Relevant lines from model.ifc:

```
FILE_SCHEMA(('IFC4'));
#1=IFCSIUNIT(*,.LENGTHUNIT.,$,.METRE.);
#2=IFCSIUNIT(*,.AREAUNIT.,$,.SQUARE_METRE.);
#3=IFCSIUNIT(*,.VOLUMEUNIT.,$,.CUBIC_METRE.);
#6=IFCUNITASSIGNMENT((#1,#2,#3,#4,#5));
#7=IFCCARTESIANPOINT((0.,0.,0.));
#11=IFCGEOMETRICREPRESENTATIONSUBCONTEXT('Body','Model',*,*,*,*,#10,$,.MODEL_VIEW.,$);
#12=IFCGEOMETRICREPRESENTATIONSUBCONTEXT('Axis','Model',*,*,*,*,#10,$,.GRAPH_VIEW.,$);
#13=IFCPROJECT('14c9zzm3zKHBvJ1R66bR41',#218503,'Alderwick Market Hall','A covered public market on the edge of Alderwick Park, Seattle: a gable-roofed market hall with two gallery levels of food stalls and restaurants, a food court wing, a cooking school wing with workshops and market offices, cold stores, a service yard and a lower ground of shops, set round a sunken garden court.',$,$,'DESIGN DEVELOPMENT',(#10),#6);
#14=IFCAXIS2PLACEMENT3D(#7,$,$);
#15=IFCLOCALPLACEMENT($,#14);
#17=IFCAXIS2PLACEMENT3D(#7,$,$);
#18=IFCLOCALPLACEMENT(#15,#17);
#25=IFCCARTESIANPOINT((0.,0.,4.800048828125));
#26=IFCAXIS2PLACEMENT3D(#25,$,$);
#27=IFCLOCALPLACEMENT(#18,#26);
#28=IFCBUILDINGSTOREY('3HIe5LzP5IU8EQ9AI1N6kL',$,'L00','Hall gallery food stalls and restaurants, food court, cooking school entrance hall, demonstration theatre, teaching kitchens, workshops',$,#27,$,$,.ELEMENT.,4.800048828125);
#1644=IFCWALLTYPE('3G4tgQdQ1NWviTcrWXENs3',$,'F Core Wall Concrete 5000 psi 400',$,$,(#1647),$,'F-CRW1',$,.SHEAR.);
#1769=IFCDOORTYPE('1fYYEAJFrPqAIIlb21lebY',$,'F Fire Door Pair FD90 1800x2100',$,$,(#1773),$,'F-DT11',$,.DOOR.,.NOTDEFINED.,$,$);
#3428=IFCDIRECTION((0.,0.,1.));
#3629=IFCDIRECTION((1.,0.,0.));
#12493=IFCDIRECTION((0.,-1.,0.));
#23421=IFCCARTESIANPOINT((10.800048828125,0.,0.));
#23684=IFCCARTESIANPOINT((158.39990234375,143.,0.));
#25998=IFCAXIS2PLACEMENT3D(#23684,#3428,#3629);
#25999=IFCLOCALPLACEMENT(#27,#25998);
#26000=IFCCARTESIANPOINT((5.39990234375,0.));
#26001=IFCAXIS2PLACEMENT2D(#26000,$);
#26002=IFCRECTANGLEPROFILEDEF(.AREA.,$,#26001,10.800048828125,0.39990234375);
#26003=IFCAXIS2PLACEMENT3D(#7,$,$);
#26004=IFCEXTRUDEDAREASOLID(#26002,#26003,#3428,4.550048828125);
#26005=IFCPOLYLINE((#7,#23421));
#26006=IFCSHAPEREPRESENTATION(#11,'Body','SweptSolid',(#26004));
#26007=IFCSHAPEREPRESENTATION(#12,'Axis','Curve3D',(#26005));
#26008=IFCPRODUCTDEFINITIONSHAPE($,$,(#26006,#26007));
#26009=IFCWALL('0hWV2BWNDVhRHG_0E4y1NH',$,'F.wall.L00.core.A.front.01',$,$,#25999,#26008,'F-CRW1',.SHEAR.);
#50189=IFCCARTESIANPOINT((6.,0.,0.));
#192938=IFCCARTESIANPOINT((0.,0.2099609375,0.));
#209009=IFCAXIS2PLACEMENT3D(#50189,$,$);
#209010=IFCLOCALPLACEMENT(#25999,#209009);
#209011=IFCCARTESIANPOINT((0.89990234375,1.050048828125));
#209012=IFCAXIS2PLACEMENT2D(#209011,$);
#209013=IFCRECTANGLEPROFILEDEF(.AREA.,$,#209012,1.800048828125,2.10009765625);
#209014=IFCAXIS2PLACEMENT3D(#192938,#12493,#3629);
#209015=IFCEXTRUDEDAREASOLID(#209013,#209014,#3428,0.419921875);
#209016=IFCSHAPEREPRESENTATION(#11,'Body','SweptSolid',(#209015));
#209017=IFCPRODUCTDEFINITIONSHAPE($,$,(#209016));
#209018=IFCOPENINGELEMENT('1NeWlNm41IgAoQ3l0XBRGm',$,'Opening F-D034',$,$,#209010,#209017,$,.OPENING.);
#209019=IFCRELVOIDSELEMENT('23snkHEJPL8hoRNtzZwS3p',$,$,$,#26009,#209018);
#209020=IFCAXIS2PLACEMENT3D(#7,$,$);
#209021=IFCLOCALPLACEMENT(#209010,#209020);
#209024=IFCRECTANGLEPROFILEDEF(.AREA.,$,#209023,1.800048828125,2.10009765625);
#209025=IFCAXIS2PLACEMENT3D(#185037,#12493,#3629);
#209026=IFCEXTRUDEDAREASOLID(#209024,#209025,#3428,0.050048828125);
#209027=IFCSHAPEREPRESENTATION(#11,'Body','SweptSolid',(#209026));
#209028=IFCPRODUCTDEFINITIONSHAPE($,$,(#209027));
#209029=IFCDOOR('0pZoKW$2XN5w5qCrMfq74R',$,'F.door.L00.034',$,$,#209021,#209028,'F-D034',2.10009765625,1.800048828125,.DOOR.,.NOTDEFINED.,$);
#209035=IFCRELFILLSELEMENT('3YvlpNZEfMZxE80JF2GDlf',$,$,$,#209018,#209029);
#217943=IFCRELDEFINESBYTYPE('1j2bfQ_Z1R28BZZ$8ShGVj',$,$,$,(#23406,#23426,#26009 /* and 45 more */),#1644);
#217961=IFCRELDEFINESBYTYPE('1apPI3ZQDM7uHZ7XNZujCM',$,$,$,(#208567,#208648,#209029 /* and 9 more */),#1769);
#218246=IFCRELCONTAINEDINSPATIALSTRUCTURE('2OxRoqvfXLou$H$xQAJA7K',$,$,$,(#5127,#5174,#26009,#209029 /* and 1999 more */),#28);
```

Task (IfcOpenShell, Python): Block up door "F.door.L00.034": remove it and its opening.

```python
import ifcopenshell
import ifcopenshell.api.feature
import ifcopenshell.api.root
import ifcopenshell.geom
import ifcopenshell.util.shape

model = ifcopenshell.open("model.ifc")
settings = ifcopenshell.geom.settings()


def volume(element):
    """Net volume in cubic metres, openings subtracted."""
    shape = ifcopenshell.geom.create_shape(settings, element)
    return ifcopenshell.util.shape.get_volume(shape.geometry)


door = model.by_guid("0pZoKW$2XN5w5qCrMfq74R")
opening = door.FillsVoids[0].RelatingOpeningElement
wall = opening.VoidsElements[0].RelatingBuildingElement
before = volume(wall)

ifcopenshell.api.root.remove_product(model, product=door)
ifcopenshell.api.feature.remove_feature(model, feature=opening)

after = volume(wall)

print(f"wall volume {before:.3f} -> {after:.3f} m3")

model.write("model_v2.ifc")
```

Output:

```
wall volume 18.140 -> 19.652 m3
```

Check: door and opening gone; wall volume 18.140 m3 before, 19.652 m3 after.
